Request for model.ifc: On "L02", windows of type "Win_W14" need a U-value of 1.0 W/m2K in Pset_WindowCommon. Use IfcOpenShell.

First a look at what the model holds.

```python
import ifcopenshell
import ifcopenshell.util.element

model = ifcopenshell.open("model.ifc")
print(model.schema)
storey = next(s for s in model.by_type("IfcBuildingStorey") if s.Name == "L02")
windows = [e for e in ifcopenshell.util.element.get_decomposition(storey) if e.is_a("IfcWindow")]
seen = {}
for e in windows:
    element_type = ifcopenshell.util.element.get_type(e)
    key = (element_type.Name if element_type != e and element_type else None, ifcopenshell.util.element.get_pset(e, "Pset_WindowCommon", "ThermalTransmittance"))
    seen[key] = seen.get(key, 0) + 1
for (name, value), count in sorted(seen.items(), key=str):
    print(count, "x", name, "|", value)
```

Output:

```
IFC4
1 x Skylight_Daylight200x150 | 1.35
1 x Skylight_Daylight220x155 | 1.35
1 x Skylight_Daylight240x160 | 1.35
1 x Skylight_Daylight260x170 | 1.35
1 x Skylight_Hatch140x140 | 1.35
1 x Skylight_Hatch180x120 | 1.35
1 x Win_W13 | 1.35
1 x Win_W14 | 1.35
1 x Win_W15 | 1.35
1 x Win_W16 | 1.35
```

```python
import ifcopenshell
import ifcopenshell.api.pset
import ifcopenshell.util.element

model = ifcopenshell.open("model.ifc")

storey = next(s for s in model.by_type("IfcBuildingStorey") if s.Name == "L02")
windows = [e for e in ifcopenshell.util.element.get_decomposition(storey) if e.is_a("IfcWindow")]

count = 0
for e in windows:
    element_type = ifcopenshell.util.element.get_type(e)
    if element_type in (None, e) or element_type.Name != "Win_W14":
        continue
    # add_pset returns the element's existing set when there is one.
    pset = ifcopenshell.api.pset.add_pset(model, product=e, name="Pset_WindowCommon")
    ifcopenshell.api.pset.edit_pset(model, pset=pset, properties={"ThermalTransmittance": 1.0})
    count += 1

print(count, "windows updated")

model.write("model_updated.ifc")
```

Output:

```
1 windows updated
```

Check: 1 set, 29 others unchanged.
